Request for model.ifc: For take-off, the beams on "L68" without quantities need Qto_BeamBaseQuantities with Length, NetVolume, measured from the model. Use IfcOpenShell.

First a look at what the model holds.

```python
import ifcopenshell
import ifcopenshell.util.element
import ifcopenshell.util.unit

model = ifcopenshell.open("model.ifc")
print(model.schema)
for unit_type in ("LENGTHUNIT", "AREAUNIT", "VOLUMEUNIT"):
    print(unit_type, ifcopenshell.util.unit.calculate_unit_scale(model, unit_type))
storey = next(s for s in model.by_type("IfcBuildingStorey") if s.Name == "L68")
beams = [e for e in ifcopenshell.util.element.get_decomposition(storey) if e.is_a("IfcBeam")]
for e in sorted(beams, key=lambda e: e.id()):
    print(e.id(), e.is_a(), e.Name, list(ifcopenshell.util.element.get_psets(e, qtos_only=True)), sep=" | ")
```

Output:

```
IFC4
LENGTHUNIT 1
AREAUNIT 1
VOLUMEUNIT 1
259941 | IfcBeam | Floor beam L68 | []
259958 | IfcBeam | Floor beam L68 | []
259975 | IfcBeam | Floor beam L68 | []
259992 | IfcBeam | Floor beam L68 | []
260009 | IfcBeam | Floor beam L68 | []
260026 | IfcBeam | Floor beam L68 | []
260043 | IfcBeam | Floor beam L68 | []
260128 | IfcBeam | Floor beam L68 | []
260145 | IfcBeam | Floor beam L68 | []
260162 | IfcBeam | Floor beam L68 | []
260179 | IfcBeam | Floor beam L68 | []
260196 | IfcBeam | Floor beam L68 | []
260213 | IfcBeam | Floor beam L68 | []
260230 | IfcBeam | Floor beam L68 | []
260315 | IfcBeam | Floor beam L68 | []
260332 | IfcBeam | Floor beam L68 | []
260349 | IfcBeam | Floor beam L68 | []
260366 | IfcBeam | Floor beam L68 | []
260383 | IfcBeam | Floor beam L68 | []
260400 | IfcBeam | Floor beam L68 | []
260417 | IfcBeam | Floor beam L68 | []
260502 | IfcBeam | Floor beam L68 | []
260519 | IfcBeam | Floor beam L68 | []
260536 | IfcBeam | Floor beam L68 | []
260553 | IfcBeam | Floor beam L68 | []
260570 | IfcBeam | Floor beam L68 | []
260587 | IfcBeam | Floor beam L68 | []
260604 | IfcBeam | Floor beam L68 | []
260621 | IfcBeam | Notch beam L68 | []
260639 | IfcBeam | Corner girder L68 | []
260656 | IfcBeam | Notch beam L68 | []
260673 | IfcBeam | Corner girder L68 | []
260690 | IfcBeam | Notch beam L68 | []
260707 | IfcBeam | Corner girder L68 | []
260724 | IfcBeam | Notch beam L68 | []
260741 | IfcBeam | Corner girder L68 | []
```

```python
import ifcopenshell
import ifcopenshell.api.pset
import ifcopenshell.geom
import ifcopenshell.util.element
import ifcopenshell.util.shape
import ifcopenshell.util.unit

model = ifcopenshell.open("model.ifc")
unit_scale = ifcopenshell.util.unit.calculate_unit_scale(model)
volume_scale = ifcopenshell.util.unit.calculate_unit_scale(model, "VOLUMEUNIT")
settings = ifcopenshell.geom.settings()

storey = next(s for s in model.by_type("IfcBuildingStorey") if s.Name == "L68")
beams = [e for e in ifcopenshell.util.element.get_decomposition(storey) if e.is_a("IfcBeam")]

for e in sorted(beams, key=lambda e: e.id()):
    if ifcopenshell.util.element.get_psets(e, qtos_only=True, should_inherit=False):
        continue
    # Geometry comes back in metres, in the element's own axes.
    shape = ifcopenshell.geom.create_shape(settings, e)
    values = {
        "Length": ifcopenshell.util.shape.get_max_xyz(shape.geometry) / unit_scale,
        "NetVolume": ifcopenshell.util.shape.get_volume(shape.geometry) / volume_scale,
    }
    qto = ifcopenshell.api.pset.add_qto(model, product=e, name="Qto_BeamBaseQuantities")
    ifcopenshell.api.pset.edit_qto(model, qto=qto, properties=values)
    print(e.id(), {k: round(v, 3) for k, v in values.items()})

model.write("model_rev.ifc")
```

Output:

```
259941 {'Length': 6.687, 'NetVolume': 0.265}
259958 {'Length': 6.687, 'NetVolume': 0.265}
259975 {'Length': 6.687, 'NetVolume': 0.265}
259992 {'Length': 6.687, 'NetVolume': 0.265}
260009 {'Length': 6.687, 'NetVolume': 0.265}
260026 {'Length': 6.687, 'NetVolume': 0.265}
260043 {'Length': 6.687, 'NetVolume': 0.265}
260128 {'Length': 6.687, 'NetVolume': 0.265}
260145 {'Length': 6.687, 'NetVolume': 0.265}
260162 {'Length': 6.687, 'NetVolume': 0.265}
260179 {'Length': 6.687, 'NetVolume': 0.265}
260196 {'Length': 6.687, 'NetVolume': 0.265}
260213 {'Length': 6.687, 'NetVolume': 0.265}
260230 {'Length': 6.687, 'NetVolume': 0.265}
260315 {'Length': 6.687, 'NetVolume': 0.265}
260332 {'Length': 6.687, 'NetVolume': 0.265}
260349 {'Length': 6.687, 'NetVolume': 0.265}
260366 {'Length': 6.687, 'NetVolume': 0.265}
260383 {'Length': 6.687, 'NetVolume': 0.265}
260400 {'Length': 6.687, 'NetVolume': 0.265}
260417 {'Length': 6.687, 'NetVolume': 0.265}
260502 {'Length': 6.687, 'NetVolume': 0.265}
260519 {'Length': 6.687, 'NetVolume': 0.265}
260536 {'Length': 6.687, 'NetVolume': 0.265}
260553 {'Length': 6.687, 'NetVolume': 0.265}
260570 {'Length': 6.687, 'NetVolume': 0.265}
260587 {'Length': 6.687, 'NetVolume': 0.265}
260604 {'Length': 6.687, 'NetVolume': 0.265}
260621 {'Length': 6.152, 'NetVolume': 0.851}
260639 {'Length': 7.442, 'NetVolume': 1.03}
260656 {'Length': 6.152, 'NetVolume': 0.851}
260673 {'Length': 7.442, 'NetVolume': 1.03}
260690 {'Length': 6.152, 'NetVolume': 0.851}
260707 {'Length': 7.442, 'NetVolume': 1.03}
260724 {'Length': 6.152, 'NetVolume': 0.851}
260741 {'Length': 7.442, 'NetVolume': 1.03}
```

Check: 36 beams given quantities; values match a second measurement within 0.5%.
